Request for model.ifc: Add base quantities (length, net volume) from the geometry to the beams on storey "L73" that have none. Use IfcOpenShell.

First a look at what the model holds.

```python
import ifcopenshell
import ifcopenshell.util.element
import ifcopenshell.util.unit

model = ifcopenshell.open("model.ifc")
print(model.schema)
for unit_type in ("LENGTHUNIT", "AREAUNIT", "VOLUMEUNIT"):
    print(unit_type, ifcopenshell.util.unit.calculate_unit_scale(model, unit_type))
storey = next(s for s in model.by_type("IfcBuildingStorey") if s.Name == "L73")
beams = [e for e in ifcopenshell.util.element.get_decomposition(storey) if e.is_a("IfcBeam")]
for e in sorted(beams, key=lambda e: e.id()):
    print(e.id(), e.is_a(), e.Name, list(ifcopenshell.util.element.get_psets(e, qtos_only=True)), sep=" | ")
```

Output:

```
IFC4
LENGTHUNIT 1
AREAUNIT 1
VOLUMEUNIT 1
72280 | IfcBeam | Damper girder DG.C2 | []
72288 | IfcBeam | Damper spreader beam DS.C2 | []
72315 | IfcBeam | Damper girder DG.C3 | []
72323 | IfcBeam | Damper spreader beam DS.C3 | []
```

```python
import ifcopenshell
import ifcopenshell.api.pset
import ifcopenshell.geom
import ifcopenshell.util.element
import ifcopenshell.util.shape
import ifcopenshell.util.unit

model = ifcopenshell.open("model.ifc")
unit_scale = ifcopenshell.util.unit.calculate_unit_scale(model)
volume_scale = ifcopenshell.util.unit.calculate_unit_scale(model, "VOLUMEUNIT")
settings = ifcopenshell.geom.settings()

storey = next(s for s in model.by_type("IfcBuildingStorey") if s.Name == "L73")
beams = [e for e in ifcopenshell.util.element.get_decomposition(storey) if e.is_a("IfcBeam")]

for e in sorted(beams, key=lambda e: e.id()):
    if ifcopenshell.util.element.get_psets(e, qtos_only=True, should_inherit=False):
        continue
    # Geometry comes back in metres, in the element's own axes.
    shape = ifcopenshell.geom.create_shape(settings, e)
    values = {
        "Length": ifcopenshell.util.shape.get_max_xyz(shape.geometry) / unit_scale,
        "NetVolume": ifcopenshell.util.shape.get_volume(shape.geometry) / volume_scale,
    }
    qto = ifcopenshell.api.pset.add_qto(model, product=e, name="Qto_BeamBaseQuantities")
    ifcopenshell.api.pset.edit_qto(model, qto=qto, properties=values)
    print(e.id(), {k: round(v, 3) for k, v in values.items()})

model.write("model_rev.ifc")
```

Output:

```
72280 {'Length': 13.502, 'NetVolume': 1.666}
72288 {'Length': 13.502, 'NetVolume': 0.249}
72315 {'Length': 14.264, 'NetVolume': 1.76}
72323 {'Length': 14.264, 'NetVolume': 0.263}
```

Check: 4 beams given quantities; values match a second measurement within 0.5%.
